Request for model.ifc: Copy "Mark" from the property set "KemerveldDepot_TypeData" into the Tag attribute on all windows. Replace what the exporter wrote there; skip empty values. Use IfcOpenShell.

First a look at what the model holds.

```python
import ifcopenshell
import ifcopenshell.util.element

model = ifcopenshell.open("model.ifc")
print(model.schema)
windows = model.by_type("IfcWindow")
print(len(windows), "windows")
for e in windows[:8]:
    source = ifcopenshell.util.element.get_pset(e, "KemerveldDepot_TypeData", "Mark")
    target = e.Tag
    print(e.id(), repr(source), repr(target), sep=" | ")
```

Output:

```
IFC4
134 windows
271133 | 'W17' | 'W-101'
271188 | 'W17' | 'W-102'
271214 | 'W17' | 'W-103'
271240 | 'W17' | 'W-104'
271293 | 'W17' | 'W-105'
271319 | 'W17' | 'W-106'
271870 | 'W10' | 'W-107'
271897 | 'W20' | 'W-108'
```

```python
import ifcopenshell
import ifcopenshell.util.element

model = ifcopenshell.open("model.ifc")

count = 0
for e in model.by_type("IfcWindow"):
    value = ifcopenshell.util.element.get_pset(e, "KemerveldDepot_TypeData", "Mark")
    current = e.Tag
    if not value or not value.strip() or current == value:
        continue
    e.Tag = value
    count += 1

print(count, "windows updated")

model.write("model_updated.ifc")
```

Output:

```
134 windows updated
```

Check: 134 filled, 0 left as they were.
